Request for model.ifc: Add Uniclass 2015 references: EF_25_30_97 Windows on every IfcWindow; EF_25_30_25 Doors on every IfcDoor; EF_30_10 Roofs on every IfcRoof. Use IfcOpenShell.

First a look at what the model holds.

```python
import ifcopenshell

model = ifcopenshell.open("model.ifc")
print(model.schema)
print("classifications:", [c.Name for c in model.by_type("IfcClassification")])
for ifc_class in ("IfcDoor", "IfcRoof", "IfcStair", "IfcWall", "IfcWindow"):
    print(ifc_class, len(model.by_type(ifc_class)))
```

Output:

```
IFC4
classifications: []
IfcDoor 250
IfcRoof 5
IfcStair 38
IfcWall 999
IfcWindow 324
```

```python
import ifcopenshell
import ifcopenshell.api.classification

model = ifcopenshell.open("model.ifc")

system = ifcopenshell.api.classification.add_classification(model, classification="Uniclass 2015")

codes = {
    "IfcWindow": ("EF_25_30_97", "Windows"),
    "IfcDoor": ("EF_25_30_25", "Doors"),
    "IfcRoof": ("EF_30_10", "Roofs"),
}
for ifc_class, (code, name) in codes.items():
    products = model.by_type(ifc_class)
    ifcopenshell.api.classification.add_reference(
        model, products=products, classification=system, identification=code, name=name
    )
    print(code, len(products))

model.write("model_rev.ifc")
```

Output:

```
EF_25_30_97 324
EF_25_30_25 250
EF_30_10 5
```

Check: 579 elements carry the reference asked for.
